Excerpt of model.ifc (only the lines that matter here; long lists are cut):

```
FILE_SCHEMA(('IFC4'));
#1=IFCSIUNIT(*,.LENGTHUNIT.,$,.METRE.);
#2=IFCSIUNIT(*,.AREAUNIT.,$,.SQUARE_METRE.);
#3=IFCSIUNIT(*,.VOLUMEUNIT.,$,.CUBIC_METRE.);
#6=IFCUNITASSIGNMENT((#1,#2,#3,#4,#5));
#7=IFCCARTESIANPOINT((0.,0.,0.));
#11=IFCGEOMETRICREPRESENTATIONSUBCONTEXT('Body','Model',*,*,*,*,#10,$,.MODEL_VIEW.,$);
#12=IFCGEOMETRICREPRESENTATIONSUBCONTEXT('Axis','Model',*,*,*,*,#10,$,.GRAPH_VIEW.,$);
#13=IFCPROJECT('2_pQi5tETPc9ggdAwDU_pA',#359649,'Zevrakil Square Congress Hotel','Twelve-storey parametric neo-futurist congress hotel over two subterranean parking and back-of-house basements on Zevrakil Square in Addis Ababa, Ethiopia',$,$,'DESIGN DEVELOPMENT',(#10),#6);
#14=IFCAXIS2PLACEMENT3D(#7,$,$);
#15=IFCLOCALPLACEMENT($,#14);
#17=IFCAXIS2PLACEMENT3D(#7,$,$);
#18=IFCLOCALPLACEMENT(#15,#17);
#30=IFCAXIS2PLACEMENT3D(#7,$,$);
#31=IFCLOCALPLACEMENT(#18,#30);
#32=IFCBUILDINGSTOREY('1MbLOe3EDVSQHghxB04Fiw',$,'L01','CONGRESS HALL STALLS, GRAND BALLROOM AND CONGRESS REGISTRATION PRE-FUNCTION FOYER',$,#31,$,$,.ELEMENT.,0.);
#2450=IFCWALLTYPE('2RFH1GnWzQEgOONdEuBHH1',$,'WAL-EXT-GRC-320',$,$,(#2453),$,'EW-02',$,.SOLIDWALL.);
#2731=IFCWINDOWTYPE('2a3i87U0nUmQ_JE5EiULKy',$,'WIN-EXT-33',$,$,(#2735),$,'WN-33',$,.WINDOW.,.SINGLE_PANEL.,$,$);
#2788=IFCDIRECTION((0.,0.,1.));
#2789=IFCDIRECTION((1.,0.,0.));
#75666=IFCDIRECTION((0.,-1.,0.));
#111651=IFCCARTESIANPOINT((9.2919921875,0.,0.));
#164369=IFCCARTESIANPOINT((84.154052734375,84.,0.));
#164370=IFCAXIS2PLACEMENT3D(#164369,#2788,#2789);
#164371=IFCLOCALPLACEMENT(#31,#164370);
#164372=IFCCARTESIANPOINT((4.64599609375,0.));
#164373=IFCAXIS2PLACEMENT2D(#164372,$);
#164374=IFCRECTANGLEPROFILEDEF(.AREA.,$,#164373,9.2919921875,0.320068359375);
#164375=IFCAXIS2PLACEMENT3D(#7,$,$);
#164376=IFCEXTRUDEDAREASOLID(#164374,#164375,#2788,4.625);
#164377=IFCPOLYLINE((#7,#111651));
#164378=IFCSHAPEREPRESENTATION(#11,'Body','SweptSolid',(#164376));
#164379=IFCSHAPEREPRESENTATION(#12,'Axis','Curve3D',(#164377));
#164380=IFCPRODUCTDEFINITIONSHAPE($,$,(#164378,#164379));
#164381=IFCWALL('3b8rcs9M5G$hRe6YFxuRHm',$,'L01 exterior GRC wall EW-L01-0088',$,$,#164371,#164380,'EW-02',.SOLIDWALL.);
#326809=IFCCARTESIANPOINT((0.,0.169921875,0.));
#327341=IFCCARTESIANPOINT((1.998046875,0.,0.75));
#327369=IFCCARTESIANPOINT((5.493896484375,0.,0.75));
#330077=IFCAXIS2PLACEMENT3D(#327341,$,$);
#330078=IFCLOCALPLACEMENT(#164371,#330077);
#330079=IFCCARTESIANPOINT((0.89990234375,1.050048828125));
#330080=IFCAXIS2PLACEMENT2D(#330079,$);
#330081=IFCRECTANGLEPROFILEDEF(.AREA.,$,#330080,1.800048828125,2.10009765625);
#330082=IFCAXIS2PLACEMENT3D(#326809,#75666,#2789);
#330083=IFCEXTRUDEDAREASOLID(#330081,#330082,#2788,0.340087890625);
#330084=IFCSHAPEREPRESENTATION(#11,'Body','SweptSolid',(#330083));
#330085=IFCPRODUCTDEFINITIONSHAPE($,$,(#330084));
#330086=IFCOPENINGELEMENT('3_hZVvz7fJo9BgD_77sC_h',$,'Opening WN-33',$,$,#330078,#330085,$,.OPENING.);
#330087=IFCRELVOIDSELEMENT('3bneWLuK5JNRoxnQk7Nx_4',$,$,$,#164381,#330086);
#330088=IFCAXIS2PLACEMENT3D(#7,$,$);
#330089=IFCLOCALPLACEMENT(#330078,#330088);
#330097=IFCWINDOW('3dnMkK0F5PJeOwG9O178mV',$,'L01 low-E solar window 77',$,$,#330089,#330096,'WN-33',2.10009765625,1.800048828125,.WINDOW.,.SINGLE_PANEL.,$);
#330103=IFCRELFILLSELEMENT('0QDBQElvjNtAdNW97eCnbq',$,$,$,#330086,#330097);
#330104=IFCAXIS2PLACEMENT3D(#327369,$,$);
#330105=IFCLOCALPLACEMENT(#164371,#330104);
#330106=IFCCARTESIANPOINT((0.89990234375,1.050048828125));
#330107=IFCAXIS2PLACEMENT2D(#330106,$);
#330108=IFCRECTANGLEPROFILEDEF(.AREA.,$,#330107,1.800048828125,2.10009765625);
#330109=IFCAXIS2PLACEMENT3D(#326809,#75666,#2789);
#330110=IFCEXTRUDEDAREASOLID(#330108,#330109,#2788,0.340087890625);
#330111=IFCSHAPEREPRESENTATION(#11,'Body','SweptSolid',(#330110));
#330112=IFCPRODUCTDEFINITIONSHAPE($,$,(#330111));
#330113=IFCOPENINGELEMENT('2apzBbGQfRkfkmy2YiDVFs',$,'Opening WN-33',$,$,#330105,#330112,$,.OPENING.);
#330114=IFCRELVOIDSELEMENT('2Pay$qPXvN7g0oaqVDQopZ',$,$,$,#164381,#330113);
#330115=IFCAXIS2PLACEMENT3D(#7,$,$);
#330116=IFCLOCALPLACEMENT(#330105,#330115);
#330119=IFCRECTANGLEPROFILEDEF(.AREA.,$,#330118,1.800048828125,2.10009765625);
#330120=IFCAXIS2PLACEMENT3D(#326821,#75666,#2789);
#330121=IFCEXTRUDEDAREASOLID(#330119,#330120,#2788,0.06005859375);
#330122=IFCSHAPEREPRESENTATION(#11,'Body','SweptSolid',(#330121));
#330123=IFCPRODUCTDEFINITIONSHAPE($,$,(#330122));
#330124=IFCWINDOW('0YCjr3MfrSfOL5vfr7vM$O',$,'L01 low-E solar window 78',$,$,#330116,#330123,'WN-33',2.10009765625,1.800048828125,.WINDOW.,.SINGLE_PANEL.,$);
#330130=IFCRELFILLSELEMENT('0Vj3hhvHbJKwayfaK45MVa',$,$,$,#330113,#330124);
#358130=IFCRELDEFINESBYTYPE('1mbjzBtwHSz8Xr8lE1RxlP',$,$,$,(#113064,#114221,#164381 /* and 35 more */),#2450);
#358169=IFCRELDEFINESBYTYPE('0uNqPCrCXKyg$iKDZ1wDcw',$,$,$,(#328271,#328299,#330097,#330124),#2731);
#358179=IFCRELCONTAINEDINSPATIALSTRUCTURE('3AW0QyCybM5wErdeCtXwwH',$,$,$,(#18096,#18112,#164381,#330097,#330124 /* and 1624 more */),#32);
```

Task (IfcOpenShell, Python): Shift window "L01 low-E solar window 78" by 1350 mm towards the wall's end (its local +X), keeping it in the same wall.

```python
import ifcopenshell
import ifcopenshell.api.geometry
import ifcopenshell.util.placement

model = ifcopenshell.open("model.ifc")

window = model.by_guid("0YCjr3MfrSfOL5vfr7vM$O")
opening = window.FillsVoids[0].RelatingOpeningElement
wall = opening.VoidsElements[0].RelatingBuildingElement

wall_matrix = ifcopenshell.util.placement.get_local_placement(wall.ObjectPlacement)
shift = wall_matrix[:3, 0] * 1.35
before = ifcopenshell.util.placement.get_local_placement(window.ObjectPlacement)[:3, 3].copy()

# The window is placed relative to its opening, so it follows when the opening moves.
matrix = ifcopenshell.util.placement.get_local_placement(opening.ObjectPlacement)
matrix[:3, 3] += shift
ifcopenshell.api.geometry.edit_object_placement(
    model, product=opening, matrix=matrix, is_si=False, should_transform_children=True
)

after = ifcopenshell.util.placement.get_local_placement(window.ObjectPlacement)[:3, 3]
print("window moved by", (after - before).round(3) + 0.0)

model.write("model_v2.ifc")
```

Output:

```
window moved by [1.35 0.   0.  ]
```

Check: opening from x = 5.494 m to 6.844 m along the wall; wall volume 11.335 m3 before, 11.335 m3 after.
